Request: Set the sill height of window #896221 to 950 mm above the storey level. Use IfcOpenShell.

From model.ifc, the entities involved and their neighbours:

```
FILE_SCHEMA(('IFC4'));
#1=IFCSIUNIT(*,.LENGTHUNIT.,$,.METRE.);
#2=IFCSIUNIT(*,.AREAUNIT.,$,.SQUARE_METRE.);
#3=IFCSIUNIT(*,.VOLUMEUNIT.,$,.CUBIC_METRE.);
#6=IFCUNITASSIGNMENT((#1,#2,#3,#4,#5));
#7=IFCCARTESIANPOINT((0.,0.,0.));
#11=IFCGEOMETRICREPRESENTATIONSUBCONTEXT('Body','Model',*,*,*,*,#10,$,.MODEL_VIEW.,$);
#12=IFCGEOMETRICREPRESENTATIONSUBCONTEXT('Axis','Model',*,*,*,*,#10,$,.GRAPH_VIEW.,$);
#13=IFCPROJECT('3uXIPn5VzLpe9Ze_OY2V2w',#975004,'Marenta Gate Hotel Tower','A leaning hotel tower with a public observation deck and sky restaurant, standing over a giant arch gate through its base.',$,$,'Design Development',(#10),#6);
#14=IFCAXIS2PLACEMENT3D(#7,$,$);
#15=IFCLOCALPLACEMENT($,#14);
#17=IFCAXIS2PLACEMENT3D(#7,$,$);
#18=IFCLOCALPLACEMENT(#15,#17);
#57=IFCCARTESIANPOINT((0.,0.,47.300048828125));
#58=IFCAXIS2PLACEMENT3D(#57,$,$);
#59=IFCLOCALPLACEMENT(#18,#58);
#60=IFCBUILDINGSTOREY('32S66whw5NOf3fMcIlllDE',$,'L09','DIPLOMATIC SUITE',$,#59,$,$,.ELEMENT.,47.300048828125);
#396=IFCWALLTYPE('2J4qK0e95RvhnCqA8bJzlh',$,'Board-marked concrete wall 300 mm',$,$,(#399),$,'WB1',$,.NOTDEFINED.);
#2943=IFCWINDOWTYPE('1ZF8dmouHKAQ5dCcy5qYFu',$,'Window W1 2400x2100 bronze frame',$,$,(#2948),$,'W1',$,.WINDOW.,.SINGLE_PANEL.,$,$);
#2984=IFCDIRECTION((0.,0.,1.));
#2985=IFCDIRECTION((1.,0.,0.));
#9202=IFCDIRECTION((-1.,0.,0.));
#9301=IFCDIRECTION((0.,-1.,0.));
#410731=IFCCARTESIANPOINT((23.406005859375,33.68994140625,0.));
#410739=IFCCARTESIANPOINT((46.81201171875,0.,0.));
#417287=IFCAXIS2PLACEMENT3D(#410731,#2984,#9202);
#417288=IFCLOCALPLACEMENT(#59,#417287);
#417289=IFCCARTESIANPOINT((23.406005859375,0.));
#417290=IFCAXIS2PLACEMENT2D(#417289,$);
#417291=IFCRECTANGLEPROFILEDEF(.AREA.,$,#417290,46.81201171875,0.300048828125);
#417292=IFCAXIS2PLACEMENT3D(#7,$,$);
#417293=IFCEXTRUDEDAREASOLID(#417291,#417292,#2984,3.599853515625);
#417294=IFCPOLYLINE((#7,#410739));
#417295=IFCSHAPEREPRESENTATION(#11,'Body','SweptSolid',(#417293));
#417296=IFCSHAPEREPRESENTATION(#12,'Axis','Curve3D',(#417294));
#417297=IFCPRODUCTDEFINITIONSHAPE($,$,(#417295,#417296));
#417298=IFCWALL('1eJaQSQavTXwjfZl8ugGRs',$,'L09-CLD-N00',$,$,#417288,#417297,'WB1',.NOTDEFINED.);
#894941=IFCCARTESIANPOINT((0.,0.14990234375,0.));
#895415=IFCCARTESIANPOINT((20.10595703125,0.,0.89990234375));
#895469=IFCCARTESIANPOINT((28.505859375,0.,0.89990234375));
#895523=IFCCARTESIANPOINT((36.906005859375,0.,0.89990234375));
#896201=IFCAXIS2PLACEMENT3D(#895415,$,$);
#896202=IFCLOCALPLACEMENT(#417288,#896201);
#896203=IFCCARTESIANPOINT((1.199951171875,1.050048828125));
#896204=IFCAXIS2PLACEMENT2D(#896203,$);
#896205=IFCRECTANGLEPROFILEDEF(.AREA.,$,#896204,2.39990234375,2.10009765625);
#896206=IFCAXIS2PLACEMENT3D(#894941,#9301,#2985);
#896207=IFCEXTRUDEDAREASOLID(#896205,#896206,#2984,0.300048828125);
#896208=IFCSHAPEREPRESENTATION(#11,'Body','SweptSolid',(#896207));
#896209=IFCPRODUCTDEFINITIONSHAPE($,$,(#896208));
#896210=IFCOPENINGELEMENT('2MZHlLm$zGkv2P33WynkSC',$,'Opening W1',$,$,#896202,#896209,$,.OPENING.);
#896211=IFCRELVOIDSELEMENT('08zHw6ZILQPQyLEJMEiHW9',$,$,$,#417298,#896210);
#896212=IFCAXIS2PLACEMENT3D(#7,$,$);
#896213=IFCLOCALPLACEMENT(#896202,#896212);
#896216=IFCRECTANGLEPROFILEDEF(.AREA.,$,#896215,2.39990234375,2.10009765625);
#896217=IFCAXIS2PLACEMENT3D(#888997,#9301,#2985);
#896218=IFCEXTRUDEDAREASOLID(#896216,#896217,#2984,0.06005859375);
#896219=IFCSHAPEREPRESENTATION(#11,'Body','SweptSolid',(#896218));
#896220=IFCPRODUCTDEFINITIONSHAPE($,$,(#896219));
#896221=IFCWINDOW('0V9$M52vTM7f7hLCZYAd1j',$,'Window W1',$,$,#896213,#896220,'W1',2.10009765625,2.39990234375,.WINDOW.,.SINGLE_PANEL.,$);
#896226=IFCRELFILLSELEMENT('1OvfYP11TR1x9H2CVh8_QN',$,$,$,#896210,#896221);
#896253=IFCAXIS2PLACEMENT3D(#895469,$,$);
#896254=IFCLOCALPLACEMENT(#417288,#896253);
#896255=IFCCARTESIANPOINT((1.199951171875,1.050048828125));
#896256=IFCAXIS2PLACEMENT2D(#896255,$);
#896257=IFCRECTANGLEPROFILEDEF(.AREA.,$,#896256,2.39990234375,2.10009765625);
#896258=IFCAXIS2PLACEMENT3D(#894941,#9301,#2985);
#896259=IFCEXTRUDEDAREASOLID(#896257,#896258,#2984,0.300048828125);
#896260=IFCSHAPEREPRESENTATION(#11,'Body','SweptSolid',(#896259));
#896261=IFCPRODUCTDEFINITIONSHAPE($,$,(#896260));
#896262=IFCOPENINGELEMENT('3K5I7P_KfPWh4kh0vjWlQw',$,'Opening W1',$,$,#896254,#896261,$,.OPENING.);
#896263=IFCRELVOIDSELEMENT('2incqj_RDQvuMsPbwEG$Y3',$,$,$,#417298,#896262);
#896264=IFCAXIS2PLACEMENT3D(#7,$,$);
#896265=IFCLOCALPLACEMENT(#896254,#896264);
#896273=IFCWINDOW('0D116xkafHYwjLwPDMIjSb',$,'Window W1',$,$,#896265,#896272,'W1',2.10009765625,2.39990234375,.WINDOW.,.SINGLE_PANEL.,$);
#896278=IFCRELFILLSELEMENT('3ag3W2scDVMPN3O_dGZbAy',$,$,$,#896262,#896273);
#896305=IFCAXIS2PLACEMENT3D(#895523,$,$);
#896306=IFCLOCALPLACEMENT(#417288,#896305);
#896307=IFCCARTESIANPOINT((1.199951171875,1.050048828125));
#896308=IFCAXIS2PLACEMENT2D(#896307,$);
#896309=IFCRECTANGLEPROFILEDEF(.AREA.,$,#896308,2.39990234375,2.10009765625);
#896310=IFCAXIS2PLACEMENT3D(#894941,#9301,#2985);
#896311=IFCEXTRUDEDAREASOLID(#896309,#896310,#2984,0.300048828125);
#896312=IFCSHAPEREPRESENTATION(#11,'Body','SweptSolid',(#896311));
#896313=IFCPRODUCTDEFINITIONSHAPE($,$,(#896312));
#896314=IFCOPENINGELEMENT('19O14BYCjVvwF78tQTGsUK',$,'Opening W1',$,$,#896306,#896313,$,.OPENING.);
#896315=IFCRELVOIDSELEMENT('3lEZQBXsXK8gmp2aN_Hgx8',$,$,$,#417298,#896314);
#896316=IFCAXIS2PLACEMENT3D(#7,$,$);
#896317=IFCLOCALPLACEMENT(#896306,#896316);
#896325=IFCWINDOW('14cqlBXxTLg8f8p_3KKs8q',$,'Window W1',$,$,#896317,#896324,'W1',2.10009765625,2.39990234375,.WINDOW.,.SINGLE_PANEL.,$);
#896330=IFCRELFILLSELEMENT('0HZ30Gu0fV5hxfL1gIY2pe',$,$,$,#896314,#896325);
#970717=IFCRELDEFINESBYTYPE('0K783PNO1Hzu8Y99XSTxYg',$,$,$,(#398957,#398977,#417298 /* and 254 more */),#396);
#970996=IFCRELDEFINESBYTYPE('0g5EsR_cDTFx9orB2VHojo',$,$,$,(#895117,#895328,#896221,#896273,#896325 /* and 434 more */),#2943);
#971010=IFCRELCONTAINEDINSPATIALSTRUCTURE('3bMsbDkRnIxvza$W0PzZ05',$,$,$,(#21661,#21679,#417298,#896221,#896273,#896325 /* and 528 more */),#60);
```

```python
import numpy as np
import ifcopenshell
import ifcopenshell.api.geometry
import ifcopenshell.geom
import ifcopenshell.util.element
import ifcopenshell.util.placement
import ifcopenshell.util.shape
import ifcopenshell.util.unit

model = ifcopenshell.open("model.ifc")
unit_scale = ifcopenshell.util.unit.calculate_unit_scale(model)

window = model.by_id(896221)
opening = window.FillsVoids[0].RelatingOpeningElement
storey = ifcopenshell.util.element.get_container(window, ifc_class="IfcBuildingStorey")
level = ifcopenshell.util.placement.get_local_placement(storey.ObjectPlacement)[2, 3]

# The opening's origin need not be at the sill, so measure its lowest point.
shape = ifcopenshell.geom.create_shape(ifcopenshell.geom.settings(), opening)
bottom = ifcopenshell.util.shape.get_shape_bottom_elevation(shape, shape.geometry) / unit_scale
dz = level + 0.95 - bottom

shift = np.array([0.0, 0.0, dz])
# The window is placed relative to its opening, so it follows when the opening moves.
matrix = ifcopenshell.util.placement.get_local_placement(opening.ObjectPlacement)
matrix[:3, 3] += shift
ifcopenshell.api.geometry.edit_object_placement(
    model, product=opening, matrix=matrix, is_si=False, should_transform_children=True
)

print(f"moved by {dz * unit_scale:+.3f} m")

model.write("model_rev.ifc")
```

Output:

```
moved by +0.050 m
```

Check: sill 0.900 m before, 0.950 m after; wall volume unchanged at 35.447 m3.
